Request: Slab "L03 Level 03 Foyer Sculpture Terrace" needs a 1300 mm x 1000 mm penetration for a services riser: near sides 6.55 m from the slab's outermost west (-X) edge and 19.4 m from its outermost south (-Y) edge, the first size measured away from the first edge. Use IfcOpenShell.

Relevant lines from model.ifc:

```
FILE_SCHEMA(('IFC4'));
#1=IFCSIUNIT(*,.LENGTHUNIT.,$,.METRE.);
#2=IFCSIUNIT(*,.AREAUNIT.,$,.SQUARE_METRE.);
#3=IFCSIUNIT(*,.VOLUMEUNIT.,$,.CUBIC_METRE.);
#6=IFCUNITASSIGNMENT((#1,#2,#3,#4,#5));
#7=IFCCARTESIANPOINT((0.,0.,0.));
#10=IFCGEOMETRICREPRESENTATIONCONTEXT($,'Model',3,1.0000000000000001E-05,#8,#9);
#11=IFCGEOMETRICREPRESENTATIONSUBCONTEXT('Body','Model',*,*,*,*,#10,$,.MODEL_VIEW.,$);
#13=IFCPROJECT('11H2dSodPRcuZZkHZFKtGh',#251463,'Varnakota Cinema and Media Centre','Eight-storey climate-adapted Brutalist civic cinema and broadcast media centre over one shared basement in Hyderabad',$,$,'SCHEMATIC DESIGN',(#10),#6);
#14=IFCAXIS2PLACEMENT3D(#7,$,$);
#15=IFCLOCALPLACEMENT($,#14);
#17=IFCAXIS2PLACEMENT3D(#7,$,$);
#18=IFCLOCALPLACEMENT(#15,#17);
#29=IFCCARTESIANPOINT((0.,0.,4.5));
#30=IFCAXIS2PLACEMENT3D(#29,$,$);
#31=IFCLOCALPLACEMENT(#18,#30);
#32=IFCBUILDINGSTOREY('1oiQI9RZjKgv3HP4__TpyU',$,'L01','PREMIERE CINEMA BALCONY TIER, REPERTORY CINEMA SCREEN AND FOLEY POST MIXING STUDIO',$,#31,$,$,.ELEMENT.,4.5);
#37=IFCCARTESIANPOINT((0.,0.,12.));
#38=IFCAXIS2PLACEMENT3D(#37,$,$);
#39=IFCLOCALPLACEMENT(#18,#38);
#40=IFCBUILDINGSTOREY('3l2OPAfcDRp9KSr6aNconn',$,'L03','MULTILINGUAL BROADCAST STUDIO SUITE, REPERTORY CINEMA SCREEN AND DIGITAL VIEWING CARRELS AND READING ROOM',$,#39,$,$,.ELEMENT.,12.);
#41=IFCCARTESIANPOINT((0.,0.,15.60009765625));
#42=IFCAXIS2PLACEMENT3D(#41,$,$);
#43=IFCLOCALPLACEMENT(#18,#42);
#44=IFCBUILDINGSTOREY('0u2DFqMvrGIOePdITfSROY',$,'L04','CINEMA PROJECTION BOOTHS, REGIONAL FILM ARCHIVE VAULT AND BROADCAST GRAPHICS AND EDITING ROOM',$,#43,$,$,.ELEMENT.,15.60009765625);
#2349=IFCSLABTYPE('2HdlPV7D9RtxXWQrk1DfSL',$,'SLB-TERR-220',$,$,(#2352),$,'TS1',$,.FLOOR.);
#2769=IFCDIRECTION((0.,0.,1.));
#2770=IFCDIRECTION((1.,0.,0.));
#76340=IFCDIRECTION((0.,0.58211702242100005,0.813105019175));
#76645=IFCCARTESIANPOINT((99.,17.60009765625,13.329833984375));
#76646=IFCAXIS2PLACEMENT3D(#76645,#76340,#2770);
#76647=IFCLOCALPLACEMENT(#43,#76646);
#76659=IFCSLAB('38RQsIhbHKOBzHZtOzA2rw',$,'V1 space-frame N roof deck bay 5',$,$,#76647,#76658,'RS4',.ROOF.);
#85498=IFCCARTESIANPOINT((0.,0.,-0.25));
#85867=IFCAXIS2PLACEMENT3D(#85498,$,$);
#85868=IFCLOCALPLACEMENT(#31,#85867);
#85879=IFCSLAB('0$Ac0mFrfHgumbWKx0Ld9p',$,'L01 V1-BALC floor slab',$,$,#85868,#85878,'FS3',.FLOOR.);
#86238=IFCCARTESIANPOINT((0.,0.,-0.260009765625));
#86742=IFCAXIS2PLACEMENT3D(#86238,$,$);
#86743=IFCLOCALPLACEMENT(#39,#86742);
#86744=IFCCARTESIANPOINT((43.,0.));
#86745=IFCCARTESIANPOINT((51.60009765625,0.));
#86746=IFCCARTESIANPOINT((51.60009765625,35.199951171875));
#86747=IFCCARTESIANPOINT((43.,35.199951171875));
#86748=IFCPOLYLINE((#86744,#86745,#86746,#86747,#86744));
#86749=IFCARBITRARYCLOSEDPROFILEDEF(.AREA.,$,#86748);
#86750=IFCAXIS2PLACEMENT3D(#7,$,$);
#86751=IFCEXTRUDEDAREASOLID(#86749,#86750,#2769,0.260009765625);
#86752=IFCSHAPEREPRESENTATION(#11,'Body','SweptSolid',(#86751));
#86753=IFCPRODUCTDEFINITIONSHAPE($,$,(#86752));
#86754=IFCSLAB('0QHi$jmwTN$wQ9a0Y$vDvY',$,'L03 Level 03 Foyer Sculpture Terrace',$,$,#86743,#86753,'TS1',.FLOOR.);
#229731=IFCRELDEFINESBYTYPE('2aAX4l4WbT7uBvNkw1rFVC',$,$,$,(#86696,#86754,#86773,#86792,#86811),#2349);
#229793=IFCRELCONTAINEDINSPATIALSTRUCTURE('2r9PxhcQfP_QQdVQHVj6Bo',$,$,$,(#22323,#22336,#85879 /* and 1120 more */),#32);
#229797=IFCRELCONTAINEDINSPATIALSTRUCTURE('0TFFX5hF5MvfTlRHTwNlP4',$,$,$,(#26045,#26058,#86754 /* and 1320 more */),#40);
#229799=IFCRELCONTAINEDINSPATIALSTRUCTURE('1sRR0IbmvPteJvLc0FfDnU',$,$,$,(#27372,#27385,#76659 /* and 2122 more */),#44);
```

```python
import numpy as np
import ifcopenshell
import ifcopenshell.api.feature
import ifcopenshell.api.geometry
import ifcopenshell.api.root
import ifcopenshell.geom
import ifcopenshell.util.placement
import ifcopenshell.util.representation
import ifcopenshell.util.shape
import ifcopenshell.util.unit

model = ifcopenshell.open("model.ifc")
unit_scale = ifcopenshell.util.unit.calculate_unit_scale(model)
settings = ifcopenshell.geom.settings()


def volume(element):
    """Net volume in cubic metres, openings subtracted."""
    shape = ifcopenshell.geom.create_shape(settings, element)
    return ifcopenshell.util.shape.get_volume(shape.geometry)


slab = model.by_guid("0QHi$jmwTN$wQ9a0Y$vDvY")
before = volume(slab)

# Extent in the slab's own axes, in metres. The edges named are its -X and -Y sides.
slab_shape = ifcopenshell.geom.create_shape(settings, slab)
vertices = ifcopenshell.util.shape.get_vertices(slab_shape.geometry)
x_min, y_min, bottom = vertices.min(axis=0)
top = vertices[:, 2].max()

opening = ifcopenshell.api.root.create_entity(model, ifc_class="IfcOpeningElement", name="Services riser opening", predefined_type="OPENING")
context = ifcopenshell.util.representation.get_context(model, "Model", "Body", "MODEL_VIEW")
width, depth = 1.3, 1
outline = [(0.0, 0.0), (width, 0.0), (width, depth), (0.0, depth), (0.0, 0.0)]
# Overshoot both faces by 50 mm so the cut is clean.
shape = ifcopenshell.api.geometry.add_slab_representation(
    model, context=context, depth=top - bottom + 0.1, polyline=outline
)
ifcopenshell.api.geometry.assign_representation(model, product=opening, representation=shape)

matrix = ifcopenshell.util.placement.get_local_placement(slab.ObjectPlacement)
matrix[:, 3] = matrix @ np.append(np.array([x_min + 6.55, y_min + 19.4, bottom - 0.05]) / unit_scale, 1.0)
ifcopenshell.api.geometry.edit_object_placement(model, product=opening, matrix=matrix, is_si=False)
ifcopenshell.api.feature.add_feature(model, feature=opening, element=slab)

after = volume(slab)

print(f"slab volume {before:.3f} -> {after:.3f} m3")

model.write("model_rev.ifc")
```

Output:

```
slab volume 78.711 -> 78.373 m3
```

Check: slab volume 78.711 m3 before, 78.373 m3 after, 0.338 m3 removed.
